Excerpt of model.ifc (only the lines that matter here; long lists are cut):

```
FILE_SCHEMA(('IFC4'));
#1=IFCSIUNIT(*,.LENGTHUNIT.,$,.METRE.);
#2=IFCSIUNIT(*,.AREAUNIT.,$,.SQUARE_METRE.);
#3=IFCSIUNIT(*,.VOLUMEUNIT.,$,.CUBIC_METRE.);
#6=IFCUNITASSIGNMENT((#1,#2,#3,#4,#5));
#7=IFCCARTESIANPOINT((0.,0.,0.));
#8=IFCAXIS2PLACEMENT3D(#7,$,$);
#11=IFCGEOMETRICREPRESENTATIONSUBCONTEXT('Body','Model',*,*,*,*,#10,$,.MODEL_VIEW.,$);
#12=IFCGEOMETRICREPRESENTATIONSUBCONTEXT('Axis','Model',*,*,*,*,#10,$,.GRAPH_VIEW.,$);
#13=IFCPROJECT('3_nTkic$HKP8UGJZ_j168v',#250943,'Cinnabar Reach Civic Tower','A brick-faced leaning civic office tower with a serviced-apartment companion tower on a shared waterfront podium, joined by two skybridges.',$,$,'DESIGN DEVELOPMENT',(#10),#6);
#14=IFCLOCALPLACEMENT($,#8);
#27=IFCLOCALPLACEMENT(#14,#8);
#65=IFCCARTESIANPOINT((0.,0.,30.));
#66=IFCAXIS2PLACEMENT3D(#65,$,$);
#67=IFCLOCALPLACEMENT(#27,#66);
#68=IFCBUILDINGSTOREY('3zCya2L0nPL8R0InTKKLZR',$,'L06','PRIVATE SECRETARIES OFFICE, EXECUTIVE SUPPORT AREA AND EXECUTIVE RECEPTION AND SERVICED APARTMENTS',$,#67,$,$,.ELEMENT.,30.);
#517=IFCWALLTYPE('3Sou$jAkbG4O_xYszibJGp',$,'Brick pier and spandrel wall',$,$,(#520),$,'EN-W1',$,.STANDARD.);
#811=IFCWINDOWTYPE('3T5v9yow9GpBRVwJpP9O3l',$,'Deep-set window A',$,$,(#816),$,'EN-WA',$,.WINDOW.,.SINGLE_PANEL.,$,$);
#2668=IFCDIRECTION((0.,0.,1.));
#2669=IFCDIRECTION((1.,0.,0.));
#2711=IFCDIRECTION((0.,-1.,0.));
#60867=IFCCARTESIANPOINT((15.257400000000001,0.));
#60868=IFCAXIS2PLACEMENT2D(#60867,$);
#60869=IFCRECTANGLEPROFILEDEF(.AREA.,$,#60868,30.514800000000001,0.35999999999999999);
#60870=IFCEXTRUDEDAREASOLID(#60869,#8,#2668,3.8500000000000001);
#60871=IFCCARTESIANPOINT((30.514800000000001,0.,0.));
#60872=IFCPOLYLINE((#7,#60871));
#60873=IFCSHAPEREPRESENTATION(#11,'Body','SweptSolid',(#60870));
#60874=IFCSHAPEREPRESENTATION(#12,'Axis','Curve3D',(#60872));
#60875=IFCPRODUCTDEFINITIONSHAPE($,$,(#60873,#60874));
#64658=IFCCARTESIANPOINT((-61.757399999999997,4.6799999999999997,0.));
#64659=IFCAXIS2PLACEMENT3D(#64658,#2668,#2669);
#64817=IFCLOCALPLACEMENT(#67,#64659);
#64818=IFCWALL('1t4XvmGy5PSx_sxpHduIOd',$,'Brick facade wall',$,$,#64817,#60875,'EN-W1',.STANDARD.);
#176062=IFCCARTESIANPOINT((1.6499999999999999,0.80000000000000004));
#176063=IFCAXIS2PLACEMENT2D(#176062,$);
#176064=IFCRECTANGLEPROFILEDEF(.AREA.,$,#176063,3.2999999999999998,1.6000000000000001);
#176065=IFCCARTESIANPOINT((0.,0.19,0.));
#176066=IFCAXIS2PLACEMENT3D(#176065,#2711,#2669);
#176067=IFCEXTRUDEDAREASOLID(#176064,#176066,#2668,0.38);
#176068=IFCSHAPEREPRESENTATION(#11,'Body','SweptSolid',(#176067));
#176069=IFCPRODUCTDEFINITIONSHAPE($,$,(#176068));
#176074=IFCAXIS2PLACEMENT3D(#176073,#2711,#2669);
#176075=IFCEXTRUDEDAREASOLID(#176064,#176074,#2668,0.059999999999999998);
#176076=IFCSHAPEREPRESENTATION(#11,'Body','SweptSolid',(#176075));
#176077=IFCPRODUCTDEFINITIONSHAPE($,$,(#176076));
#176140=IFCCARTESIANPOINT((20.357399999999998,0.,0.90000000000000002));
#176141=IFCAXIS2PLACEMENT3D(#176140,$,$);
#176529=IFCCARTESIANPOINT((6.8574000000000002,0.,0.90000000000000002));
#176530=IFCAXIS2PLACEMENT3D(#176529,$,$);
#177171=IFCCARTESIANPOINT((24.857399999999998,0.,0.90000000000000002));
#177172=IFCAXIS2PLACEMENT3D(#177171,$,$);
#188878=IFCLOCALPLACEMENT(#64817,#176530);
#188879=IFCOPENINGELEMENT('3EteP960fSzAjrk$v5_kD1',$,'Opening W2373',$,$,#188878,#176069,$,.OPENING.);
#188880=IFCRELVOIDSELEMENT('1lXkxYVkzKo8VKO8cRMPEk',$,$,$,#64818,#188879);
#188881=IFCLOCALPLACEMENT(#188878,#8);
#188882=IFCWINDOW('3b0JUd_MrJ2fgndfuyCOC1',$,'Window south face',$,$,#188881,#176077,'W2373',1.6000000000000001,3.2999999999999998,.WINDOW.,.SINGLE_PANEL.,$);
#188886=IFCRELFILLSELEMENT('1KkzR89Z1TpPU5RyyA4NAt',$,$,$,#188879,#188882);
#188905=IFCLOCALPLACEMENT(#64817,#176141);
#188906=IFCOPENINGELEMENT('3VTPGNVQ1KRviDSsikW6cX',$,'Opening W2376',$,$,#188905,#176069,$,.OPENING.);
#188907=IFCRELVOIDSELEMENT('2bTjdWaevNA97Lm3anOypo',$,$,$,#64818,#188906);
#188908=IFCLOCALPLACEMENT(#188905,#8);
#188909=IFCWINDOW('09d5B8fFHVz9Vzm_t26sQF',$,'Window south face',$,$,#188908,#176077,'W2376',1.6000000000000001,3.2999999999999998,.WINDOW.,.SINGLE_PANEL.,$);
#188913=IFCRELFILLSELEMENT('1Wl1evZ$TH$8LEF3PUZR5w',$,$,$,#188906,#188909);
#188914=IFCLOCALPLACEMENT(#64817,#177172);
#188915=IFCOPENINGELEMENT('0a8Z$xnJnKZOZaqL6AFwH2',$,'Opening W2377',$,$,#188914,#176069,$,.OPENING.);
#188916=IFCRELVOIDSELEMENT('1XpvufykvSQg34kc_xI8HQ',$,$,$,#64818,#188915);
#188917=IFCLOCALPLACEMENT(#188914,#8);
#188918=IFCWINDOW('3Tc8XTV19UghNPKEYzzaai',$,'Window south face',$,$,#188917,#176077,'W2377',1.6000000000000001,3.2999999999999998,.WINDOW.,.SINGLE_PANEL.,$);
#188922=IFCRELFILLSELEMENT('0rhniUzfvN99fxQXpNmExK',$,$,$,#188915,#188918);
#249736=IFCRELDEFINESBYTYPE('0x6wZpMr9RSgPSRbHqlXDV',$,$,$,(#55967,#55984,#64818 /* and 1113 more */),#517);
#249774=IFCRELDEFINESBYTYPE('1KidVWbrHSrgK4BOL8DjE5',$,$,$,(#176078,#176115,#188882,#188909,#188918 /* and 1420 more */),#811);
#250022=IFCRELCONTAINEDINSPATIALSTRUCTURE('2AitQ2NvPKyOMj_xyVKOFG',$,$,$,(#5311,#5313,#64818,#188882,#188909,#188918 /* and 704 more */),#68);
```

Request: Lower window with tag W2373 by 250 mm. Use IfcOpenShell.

```python
import numpy as np
import ifcopenshell
import ifcopenshell.api.geometry
import ifcopenshell.util.placement
import ifcopenshell.util.unit

model = ifcopenshell.open("model.ifc")
unit_scale = ifcopenshell.util.unit.calculate_unit_scale(model)

window = model.by_id(188882)
opening = window.FillsVoids[0].RelatingOpeningElement
dz = -0.25 / unit_scale

shift = np.array([0.0, 0.0, dz])
# The window is placed relative to its opening, so it follows when the opening moves.
matrix = ifcopenshell.util.placement.get_local_placement(opening.ObjectPlacement)
matrix[:3, 3] += shift
ifcopenshell.api.geometry.edit_object_placement(
    model, product=opening, matrix=matrix, is_si=False, should_transform_children=True
)

print(f"moved by {dz * unit_scale:+.3f} m")

model.write("model_edited.ifc")
```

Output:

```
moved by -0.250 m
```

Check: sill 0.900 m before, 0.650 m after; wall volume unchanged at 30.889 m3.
